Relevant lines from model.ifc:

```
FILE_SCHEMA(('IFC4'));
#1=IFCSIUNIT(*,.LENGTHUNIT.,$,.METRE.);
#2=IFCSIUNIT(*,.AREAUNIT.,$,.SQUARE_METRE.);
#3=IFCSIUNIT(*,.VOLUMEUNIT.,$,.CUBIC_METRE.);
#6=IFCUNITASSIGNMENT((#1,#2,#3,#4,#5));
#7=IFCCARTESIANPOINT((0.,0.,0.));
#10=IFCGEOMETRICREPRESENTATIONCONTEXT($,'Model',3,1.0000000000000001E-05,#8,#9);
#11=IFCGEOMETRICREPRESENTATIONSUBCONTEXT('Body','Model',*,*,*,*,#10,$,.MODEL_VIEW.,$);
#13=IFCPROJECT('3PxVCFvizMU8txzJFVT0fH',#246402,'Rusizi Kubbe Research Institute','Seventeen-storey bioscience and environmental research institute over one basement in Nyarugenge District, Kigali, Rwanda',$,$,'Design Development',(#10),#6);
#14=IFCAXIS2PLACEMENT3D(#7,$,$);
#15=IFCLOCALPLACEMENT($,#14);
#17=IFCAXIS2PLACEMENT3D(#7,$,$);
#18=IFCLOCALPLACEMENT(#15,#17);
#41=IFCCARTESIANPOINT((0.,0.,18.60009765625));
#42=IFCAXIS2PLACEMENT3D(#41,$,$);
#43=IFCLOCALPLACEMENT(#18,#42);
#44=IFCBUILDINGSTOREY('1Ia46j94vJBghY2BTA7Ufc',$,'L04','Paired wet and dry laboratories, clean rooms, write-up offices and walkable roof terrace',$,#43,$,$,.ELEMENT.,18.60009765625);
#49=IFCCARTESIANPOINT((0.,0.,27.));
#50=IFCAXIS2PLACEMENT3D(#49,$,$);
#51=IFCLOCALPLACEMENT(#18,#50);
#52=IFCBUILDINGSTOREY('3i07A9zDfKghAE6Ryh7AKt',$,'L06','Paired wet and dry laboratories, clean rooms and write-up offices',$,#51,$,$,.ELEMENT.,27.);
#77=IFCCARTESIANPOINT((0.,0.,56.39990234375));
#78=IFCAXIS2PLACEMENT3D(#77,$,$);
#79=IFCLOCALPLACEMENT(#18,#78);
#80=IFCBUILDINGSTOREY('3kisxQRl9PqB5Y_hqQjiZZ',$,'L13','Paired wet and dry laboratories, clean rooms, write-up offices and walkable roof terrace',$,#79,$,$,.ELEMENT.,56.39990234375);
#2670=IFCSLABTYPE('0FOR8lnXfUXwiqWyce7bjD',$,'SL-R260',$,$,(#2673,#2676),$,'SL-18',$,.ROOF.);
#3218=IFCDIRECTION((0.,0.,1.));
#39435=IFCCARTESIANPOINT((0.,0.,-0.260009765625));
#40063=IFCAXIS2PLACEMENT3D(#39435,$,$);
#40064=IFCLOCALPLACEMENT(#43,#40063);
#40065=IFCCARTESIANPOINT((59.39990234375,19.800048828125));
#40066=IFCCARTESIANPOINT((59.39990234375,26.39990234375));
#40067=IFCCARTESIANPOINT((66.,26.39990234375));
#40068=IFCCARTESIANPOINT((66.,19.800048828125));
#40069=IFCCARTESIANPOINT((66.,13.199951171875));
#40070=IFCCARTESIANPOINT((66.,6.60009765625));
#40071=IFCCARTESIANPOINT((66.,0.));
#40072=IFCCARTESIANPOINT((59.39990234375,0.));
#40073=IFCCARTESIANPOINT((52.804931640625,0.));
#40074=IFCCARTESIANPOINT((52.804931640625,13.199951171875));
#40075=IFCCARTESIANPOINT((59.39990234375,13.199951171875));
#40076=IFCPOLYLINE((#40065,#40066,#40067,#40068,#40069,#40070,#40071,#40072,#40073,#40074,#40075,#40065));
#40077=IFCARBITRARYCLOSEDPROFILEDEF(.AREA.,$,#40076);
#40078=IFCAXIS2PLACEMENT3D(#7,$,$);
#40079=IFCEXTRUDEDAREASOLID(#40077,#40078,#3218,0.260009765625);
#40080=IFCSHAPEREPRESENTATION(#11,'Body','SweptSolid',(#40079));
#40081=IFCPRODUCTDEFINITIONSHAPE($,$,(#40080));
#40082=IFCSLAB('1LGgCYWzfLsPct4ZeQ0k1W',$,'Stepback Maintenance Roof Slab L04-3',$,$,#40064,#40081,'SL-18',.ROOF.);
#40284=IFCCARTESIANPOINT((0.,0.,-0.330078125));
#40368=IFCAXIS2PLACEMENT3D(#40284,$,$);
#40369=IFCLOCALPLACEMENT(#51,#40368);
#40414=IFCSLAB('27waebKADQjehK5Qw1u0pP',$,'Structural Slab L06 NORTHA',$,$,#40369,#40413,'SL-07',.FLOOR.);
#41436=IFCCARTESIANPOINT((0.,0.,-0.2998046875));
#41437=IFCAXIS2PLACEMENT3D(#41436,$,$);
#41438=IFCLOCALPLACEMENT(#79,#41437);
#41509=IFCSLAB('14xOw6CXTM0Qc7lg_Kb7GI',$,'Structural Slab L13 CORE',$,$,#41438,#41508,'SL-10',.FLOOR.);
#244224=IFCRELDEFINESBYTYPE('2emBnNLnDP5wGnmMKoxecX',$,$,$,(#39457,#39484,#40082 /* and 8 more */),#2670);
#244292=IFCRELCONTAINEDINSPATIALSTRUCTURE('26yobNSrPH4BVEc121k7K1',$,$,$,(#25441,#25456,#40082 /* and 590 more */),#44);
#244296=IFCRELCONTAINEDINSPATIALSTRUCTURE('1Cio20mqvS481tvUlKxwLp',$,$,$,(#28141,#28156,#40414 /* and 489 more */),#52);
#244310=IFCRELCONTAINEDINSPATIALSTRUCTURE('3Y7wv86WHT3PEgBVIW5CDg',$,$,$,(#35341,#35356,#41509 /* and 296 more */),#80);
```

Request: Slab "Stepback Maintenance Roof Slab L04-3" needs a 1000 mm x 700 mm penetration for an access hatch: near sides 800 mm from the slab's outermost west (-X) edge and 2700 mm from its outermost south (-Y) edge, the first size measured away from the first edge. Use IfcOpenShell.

```python
import numpy as np
import ifcopenshell
import ifcopenshell.api.feature
import ifcopenshell.api.geometry
import ifcopenshell.api.root
import ifcopenshell.geom
import ifcopenshell.util.placement
import ifcopenshell.util.representation
import ifcopenshell.util.shape
import ifcopenshell.util.unit

model = ifcopenshell.open("model.ifc")
unit_scale = ifcopenshell.util.unit.calculate_unit_scale(model)
settings = ifcopenshell.geom.settings()


def volume(element):
    """Net volume in cubic metres, openings subtracted."""
    shape = ifcopenshell.geom.create_shape(settings, element)
    return ifcopenshell.util.shape.get_volume(shape.geometry)


slab = model.by_guid("1LGgCYWzfLsPct4ZeQ0k1W")
before = volume(slab)

# Extent in the slab's own axes, in metres. The edges named are its -X and -Y sides.
slab_shape = ifcopenshell.geom.create_shape(settings, slab)
vertices = ifcopenshell.util.shape.get_vertices(slab_shape.geometry)
x_min, y_min, bottom = vertices.min(axis=0)
top = vertices[:, 2].max()

opening = ifcopenshell.api.root.create_entity(model, ifc_class="IfcOpeningElement", name="Access hatch opening", predefined_type="OPENING")
context = ifcopenshell.util.representation.get_context(model, "Model", "Body", "MODEL_VIEW")
width, depth = 1, 0.7
outline = [(0.0, 0.0), (width, 0.0), (width, depth), (0.0, depth), (0.0, 0.0)]
# Overshoot both faces by 50 mm so the cut is clean.
shape = ifcopenshell.api.geometry.add_slab_representation(
    model, context=context, depth=top - bottom + 0.1, polyline=outline
)
ifcopenshell.api.geometry.assign_representation(model, product=opening, representation=shape)

matrix = ifcopenshell.util.placement.get_local_placement(slab.ObjectPlacement)
matrix[:, 3] = matrix @ np.append(np.array([x_min + 0.8, y_min + 2.7, bottom - 0.05]) / unit_scale, 1.0)
ifcopenshell.api.geometry.edit_object_placement(model, product=opening, matrix=matrix, is_si=False)
ifcopenshell.api.feature.add_feature(model, feature=opening, element=slab)

after = volume(slab)

print(f"slab volume {before:.3f} -> {after:.3f} m3")

model.write("model-out.ifc")
```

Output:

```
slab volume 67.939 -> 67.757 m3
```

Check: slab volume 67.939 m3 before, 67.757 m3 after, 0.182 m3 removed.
